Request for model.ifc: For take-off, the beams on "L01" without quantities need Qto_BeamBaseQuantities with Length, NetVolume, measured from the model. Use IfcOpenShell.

First a look at what the model holds.

```python
import ifcopenshell
import ifcopenshell.util.element
import ifcopenshell.util.unit

model = ifcopenshell.open("model.ifc")
print(model.schema)
for unit_type in ("LENGTHUNIT", "AREAUNIT", "VOLUMEUNIT"):
    print(unit_type, ifcopenshell.util.unit.calculate_unit_scale(model, unit_type))
storey = next(s for s in model.by_type("IfcBuildingStorey") if s.Name == "L01")
beams = [e for e in ifcopenshell.util.element.get_decomposition(storey) if e.is_a("IfcBeam")]
for e in sorted(beams, key=lambda e: e.id()):
    print(e.id(), e.is_a(), e.Name, list(ifcopenshell.util.element.get_psets(e, qtos_only=True)), sep=" | ")
```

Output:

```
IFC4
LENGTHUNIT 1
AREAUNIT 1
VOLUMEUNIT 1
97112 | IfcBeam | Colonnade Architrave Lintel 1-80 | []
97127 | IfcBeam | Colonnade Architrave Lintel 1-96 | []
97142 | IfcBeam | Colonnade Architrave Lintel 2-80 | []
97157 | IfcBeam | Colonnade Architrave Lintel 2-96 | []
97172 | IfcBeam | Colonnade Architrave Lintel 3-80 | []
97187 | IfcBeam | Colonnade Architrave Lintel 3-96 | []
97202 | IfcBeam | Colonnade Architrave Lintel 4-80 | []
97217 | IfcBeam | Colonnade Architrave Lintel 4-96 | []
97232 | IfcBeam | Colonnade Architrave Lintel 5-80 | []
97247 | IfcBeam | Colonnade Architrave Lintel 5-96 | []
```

```python
import ifcopenshell
import ifcopenshell.api.pset
import ifcopenshell.geom
import ifcopenshell.util.element
import ifcopenshell.util.shape
import ifcopenshell.util.unit

model = ifcopenshell.open("model.ifc")
unit_scale = ifcopenshell.util.unit.calculate_unit_scale(model)
volume_scale = ifcopenshell.util.unit.calculate_unit_scale(model, "VOLUMEUNIT")
settings = ifcopenshell.geom.settings()

storey = next(s for s in model.by_type("IfcBuildingStorey") if s.Name == "L01")
beams = [e for e in ifcopenshell.util.element.get_decomposition(storey) if e.is_a("IfcBeam")]

for e in sorted(beams, key=lambda e: e.id()):
    if ifcopenshell.util.element.get_psets(e, qtos_only=True, should_inherit=False):
        continue
    # Geometry comes back in metres, in the element's own axes.
    shape = ifcopenshell.geom.create_shape(settings, e)
    values = {
        "Length": ifcopenshell.util.shape.get_max_xyz(shape.geometry) / unit_scale,
        "NetVolume": ifcopenshell.util.shape.get_volume(shape.geometry) / volume_scale,
    }
    qto = ifcopenshell.api.pset.add_qto(model, product=e, name="Qto_BeamBaseQuantities")
    ifcopenshell.api.pset.edit_qto(model, qto=qto, properties=values)
    print(e.id(), {k: round(v, 3) for k, v in values.items()})

model.write("model_rev.ifc")
```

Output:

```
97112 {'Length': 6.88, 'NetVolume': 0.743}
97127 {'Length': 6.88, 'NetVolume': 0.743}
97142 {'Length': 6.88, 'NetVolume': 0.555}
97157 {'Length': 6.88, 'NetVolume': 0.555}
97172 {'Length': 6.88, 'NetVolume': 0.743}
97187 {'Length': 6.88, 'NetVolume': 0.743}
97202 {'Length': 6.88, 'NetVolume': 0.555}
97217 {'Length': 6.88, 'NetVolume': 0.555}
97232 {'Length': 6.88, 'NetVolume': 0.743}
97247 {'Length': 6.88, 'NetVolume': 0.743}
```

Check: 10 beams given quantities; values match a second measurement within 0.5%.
